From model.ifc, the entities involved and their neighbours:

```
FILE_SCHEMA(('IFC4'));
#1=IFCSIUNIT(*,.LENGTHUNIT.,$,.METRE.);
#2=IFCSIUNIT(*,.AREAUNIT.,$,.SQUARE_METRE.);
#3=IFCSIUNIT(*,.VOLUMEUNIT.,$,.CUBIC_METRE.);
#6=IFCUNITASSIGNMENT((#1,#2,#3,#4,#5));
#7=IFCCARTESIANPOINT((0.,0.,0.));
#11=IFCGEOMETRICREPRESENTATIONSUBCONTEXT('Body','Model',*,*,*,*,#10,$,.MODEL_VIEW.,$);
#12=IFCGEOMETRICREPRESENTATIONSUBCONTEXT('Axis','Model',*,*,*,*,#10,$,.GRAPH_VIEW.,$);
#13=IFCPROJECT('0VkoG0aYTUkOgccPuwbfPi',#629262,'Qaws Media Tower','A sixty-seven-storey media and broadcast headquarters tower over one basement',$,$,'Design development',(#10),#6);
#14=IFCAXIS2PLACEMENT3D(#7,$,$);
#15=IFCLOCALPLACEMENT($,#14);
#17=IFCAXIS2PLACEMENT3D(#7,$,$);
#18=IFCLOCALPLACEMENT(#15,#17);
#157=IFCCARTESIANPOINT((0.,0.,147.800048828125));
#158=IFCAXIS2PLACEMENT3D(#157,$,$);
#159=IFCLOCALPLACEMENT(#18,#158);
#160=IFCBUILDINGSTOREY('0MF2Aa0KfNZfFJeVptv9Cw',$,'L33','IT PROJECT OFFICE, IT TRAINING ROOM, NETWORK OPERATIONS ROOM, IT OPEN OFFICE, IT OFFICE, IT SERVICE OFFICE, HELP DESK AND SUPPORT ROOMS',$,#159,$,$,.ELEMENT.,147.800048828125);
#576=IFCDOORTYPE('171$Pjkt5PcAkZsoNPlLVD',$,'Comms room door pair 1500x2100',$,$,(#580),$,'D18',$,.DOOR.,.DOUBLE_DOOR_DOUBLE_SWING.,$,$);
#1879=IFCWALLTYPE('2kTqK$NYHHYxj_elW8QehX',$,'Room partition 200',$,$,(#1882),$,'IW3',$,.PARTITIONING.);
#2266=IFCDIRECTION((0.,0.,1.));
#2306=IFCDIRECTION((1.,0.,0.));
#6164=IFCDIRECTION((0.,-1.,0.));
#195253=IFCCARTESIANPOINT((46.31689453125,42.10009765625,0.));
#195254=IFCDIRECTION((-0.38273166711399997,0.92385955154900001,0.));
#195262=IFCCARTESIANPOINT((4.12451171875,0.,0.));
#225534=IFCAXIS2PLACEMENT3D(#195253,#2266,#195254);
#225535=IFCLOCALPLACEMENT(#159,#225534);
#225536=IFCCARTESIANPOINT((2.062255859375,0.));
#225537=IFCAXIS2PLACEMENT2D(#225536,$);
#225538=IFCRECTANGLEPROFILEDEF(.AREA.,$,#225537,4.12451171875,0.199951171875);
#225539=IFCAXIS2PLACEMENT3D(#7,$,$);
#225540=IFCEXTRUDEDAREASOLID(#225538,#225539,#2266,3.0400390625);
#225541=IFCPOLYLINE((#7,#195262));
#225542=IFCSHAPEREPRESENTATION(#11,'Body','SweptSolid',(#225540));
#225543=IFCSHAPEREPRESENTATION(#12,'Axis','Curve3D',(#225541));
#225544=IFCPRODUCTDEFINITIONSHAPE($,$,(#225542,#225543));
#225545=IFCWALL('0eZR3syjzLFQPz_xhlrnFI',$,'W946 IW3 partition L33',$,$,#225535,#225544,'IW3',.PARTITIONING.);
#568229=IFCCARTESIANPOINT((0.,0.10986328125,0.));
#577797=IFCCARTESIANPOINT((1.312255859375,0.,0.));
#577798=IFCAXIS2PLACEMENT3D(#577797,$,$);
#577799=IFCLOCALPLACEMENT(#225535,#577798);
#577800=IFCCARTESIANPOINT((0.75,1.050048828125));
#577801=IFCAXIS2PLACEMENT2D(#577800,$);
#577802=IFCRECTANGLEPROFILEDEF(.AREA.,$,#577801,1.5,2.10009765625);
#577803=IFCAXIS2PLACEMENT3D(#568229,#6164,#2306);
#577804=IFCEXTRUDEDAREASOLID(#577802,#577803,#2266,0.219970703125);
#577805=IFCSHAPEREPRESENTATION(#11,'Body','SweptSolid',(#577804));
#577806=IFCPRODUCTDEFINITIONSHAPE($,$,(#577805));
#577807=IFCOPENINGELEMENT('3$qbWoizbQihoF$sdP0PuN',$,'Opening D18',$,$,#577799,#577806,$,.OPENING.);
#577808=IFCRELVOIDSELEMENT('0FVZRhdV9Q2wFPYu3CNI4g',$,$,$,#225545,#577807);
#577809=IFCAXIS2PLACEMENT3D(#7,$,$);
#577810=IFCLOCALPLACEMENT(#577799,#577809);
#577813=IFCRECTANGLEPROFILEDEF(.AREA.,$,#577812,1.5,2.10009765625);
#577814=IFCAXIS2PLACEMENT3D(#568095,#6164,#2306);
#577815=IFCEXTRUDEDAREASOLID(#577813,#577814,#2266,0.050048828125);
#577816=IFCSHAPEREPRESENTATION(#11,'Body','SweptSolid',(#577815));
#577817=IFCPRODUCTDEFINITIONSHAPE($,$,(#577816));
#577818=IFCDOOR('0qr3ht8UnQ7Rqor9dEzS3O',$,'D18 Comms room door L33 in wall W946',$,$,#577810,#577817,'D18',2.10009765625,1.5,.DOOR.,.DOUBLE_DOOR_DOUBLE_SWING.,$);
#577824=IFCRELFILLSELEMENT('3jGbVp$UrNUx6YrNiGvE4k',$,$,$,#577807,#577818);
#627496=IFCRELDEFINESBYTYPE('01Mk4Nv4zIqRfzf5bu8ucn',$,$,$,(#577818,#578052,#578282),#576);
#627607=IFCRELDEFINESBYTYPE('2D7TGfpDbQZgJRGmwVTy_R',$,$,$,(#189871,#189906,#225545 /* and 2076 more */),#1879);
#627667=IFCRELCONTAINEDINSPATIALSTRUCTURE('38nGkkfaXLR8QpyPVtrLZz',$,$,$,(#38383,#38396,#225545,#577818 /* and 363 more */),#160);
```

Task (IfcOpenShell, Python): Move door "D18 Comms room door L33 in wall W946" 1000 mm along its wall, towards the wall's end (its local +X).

```python
import ifcopenshell
import ifcopenshell.api.geometry
import ifcopenshell.util.placement

model = ifcopenshell.open("model.ifc")

door = model.by_id(577818)
opening = door.FillsVoids[0].RelatingOpeningElement
wall = opening.VoidsElements[0].RelatingBuildingElement

wall_matrix = ifcopenshell.util.placement.get_local_placement(wall.ObjectPlacement)
shift = wall_matrix[:3, 0] * 1.0
before = ifcopenshell.util.placement.get_local_placement(door.ObjectPlacement)[:3, 3].copy()

# The door is placed relative to its opening, so it follows when the opening moves.
matrix = ifcopenshell.util.placement.get_local_placement(opening.ObjectPlacement)
matrix[:3, 3] += shift
ifcopenshell.api.geometry.edit_object_placement(
    model, product=opening, matrix=matrix, is_si=False, should_transform_children=True
)

after = ifcopenshell.util.placement.get_local_placement(door.ObjectPlacement)[:3, 3]
print("door moved by", (after - before).round(3) + 0.0)

model.write("model_edited.ifc")
```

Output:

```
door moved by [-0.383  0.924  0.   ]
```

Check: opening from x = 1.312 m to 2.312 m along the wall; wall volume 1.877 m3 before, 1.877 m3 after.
